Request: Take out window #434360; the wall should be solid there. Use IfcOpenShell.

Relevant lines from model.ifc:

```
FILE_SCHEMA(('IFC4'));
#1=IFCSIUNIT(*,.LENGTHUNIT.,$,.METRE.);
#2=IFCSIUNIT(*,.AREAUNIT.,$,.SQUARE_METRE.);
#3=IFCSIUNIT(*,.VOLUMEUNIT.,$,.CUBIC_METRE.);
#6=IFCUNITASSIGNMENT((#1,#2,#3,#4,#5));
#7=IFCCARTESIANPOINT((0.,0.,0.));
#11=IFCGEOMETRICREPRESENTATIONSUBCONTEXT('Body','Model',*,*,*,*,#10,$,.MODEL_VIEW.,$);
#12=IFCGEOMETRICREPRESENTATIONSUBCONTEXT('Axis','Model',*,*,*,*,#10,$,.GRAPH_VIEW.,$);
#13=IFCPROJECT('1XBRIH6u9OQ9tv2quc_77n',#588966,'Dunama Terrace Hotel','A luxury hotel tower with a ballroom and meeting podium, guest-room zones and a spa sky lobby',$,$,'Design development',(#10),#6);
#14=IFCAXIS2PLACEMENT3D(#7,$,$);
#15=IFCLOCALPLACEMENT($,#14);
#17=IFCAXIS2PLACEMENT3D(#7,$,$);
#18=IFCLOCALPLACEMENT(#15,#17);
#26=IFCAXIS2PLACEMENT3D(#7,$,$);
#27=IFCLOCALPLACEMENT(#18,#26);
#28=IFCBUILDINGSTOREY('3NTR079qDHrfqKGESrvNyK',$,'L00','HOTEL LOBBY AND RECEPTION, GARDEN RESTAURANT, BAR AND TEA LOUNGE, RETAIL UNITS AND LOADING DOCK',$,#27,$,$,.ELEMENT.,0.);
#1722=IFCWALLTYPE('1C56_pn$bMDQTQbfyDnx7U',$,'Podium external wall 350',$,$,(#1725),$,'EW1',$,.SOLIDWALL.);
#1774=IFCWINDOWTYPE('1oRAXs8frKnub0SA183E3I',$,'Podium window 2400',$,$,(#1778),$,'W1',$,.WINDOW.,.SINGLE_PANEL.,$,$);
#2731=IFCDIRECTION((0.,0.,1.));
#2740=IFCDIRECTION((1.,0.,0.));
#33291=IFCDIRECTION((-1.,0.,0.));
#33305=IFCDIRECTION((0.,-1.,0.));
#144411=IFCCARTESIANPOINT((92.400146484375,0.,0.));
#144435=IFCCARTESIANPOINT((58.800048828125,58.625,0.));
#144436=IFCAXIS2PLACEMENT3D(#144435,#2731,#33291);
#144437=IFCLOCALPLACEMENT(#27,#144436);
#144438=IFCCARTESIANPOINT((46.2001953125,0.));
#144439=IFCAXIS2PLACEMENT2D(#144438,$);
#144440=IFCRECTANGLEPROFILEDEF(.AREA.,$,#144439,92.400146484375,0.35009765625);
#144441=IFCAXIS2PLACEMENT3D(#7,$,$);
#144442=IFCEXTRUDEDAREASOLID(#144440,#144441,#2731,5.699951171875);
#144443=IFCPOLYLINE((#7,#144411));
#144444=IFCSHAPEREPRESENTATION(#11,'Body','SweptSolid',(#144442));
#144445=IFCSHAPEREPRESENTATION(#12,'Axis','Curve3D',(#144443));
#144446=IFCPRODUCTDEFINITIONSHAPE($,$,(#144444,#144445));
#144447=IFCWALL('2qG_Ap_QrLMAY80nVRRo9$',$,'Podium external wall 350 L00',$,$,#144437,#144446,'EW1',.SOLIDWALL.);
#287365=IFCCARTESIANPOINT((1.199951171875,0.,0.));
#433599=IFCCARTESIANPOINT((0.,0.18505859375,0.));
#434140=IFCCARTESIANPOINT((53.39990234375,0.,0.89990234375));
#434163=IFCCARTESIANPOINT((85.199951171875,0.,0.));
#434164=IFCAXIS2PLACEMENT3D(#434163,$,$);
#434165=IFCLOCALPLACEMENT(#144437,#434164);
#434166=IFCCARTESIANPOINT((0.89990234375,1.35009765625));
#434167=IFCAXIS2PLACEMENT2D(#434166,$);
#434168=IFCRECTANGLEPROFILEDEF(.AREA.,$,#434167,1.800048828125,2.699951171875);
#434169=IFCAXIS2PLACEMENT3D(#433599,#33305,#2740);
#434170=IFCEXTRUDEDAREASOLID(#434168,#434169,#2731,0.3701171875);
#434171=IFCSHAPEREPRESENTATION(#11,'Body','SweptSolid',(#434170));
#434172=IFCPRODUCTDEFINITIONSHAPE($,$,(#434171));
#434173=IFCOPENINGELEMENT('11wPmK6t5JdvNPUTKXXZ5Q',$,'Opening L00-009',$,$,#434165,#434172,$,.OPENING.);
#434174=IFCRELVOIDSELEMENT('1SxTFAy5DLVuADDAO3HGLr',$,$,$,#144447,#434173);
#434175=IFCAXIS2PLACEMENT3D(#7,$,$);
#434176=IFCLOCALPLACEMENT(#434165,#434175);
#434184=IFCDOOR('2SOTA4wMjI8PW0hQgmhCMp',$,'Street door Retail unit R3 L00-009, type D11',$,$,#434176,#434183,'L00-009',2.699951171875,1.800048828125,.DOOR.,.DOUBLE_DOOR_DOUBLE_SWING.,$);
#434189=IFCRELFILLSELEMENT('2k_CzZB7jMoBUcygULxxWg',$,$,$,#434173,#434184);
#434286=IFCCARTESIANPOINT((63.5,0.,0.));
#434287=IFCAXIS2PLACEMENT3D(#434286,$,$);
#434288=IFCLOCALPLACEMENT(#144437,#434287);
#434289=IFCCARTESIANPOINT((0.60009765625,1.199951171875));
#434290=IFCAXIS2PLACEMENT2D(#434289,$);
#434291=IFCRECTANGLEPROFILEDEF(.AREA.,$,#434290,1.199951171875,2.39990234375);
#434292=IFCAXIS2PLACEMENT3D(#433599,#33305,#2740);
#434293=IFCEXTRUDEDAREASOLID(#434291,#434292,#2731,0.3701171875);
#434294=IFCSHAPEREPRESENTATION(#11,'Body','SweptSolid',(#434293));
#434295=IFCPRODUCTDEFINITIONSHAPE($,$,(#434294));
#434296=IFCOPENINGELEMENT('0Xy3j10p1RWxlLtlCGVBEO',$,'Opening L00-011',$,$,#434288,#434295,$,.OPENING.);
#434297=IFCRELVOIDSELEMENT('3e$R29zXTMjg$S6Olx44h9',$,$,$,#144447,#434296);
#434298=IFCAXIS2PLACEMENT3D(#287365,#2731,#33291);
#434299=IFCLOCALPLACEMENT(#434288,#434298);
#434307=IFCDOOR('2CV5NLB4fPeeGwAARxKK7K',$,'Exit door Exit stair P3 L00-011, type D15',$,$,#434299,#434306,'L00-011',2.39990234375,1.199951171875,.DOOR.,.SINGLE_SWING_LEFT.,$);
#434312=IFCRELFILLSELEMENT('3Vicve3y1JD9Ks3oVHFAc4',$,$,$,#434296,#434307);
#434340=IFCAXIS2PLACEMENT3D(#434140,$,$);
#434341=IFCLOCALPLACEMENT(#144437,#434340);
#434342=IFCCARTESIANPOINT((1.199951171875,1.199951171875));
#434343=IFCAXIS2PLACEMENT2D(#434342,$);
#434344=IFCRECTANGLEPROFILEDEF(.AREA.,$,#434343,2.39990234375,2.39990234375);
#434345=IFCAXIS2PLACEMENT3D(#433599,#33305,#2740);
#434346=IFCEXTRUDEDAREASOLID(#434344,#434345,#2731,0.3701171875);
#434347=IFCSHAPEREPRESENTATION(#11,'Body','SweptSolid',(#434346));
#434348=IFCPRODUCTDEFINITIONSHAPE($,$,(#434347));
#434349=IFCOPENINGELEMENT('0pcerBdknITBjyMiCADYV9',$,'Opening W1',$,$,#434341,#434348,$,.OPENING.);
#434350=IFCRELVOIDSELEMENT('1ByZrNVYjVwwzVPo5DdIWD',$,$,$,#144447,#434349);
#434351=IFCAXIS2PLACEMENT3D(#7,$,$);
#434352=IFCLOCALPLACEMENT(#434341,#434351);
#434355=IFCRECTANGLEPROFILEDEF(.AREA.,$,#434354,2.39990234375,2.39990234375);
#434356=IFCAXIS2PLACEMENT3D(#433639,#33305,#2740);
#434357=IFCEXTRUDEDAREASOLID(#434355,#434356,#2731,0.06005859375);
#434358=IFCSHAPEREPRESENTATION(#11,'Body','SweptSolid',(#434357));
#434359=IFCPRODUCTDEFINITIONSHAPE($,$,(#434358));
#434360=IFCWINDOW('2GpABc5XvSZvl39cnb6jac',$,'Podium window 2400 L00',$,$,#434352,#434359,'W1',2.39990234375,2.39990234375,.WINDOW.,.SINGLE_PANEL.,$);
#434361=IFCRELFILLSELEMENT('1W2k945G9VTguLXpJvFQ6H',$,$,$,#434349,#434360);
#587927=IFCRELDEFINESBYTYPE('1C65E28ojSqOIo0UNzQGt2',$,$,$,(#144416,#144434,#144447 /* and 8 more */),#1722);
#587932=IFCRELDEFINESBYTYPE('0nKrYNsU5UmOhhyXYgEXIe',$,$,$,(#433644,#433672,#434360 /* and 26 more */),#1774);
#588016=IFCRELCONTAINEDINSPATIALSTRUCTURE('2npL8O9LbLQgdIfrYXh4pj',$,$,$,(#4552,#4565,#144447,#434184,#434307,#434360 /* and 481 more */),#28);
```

```python
import ifcopenshell
import ifcopenshell.api.feature
import ifcopenshell.api.root
import ifcopenshell.geom
import ifcopenshell.util.shape

model = ifcopenshell.open("model.ifc")
settings = ifcopenshell.geom.settings()


def volume(element):
    """Net volume in cubic metres, openings subtracted."""
    shape = ifcopenshell.geom.create_shape(settings, element)
    return ifcopenshell.util.shape.get_volume(shape.geometry)


window = model.by_id(434360)
opening = window.FillsVoids[0].RelatingOpeningElement
wall = opening.VoidsElements[0].RelatingBuildingElement
before = volume(wall)

ifcopenshell.api.root.remove_product(model, product=window)
ifcopenshell.api.feature.remove_feature(model, feature=opening)

after = volume(wall)

print(f"wall volume {before:.3f} -> {after:.3f} m3")

model.write("model_updated.ifc")
```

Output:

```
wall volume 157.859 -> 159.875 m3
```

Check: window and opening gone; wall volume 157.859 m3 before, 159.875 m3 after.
